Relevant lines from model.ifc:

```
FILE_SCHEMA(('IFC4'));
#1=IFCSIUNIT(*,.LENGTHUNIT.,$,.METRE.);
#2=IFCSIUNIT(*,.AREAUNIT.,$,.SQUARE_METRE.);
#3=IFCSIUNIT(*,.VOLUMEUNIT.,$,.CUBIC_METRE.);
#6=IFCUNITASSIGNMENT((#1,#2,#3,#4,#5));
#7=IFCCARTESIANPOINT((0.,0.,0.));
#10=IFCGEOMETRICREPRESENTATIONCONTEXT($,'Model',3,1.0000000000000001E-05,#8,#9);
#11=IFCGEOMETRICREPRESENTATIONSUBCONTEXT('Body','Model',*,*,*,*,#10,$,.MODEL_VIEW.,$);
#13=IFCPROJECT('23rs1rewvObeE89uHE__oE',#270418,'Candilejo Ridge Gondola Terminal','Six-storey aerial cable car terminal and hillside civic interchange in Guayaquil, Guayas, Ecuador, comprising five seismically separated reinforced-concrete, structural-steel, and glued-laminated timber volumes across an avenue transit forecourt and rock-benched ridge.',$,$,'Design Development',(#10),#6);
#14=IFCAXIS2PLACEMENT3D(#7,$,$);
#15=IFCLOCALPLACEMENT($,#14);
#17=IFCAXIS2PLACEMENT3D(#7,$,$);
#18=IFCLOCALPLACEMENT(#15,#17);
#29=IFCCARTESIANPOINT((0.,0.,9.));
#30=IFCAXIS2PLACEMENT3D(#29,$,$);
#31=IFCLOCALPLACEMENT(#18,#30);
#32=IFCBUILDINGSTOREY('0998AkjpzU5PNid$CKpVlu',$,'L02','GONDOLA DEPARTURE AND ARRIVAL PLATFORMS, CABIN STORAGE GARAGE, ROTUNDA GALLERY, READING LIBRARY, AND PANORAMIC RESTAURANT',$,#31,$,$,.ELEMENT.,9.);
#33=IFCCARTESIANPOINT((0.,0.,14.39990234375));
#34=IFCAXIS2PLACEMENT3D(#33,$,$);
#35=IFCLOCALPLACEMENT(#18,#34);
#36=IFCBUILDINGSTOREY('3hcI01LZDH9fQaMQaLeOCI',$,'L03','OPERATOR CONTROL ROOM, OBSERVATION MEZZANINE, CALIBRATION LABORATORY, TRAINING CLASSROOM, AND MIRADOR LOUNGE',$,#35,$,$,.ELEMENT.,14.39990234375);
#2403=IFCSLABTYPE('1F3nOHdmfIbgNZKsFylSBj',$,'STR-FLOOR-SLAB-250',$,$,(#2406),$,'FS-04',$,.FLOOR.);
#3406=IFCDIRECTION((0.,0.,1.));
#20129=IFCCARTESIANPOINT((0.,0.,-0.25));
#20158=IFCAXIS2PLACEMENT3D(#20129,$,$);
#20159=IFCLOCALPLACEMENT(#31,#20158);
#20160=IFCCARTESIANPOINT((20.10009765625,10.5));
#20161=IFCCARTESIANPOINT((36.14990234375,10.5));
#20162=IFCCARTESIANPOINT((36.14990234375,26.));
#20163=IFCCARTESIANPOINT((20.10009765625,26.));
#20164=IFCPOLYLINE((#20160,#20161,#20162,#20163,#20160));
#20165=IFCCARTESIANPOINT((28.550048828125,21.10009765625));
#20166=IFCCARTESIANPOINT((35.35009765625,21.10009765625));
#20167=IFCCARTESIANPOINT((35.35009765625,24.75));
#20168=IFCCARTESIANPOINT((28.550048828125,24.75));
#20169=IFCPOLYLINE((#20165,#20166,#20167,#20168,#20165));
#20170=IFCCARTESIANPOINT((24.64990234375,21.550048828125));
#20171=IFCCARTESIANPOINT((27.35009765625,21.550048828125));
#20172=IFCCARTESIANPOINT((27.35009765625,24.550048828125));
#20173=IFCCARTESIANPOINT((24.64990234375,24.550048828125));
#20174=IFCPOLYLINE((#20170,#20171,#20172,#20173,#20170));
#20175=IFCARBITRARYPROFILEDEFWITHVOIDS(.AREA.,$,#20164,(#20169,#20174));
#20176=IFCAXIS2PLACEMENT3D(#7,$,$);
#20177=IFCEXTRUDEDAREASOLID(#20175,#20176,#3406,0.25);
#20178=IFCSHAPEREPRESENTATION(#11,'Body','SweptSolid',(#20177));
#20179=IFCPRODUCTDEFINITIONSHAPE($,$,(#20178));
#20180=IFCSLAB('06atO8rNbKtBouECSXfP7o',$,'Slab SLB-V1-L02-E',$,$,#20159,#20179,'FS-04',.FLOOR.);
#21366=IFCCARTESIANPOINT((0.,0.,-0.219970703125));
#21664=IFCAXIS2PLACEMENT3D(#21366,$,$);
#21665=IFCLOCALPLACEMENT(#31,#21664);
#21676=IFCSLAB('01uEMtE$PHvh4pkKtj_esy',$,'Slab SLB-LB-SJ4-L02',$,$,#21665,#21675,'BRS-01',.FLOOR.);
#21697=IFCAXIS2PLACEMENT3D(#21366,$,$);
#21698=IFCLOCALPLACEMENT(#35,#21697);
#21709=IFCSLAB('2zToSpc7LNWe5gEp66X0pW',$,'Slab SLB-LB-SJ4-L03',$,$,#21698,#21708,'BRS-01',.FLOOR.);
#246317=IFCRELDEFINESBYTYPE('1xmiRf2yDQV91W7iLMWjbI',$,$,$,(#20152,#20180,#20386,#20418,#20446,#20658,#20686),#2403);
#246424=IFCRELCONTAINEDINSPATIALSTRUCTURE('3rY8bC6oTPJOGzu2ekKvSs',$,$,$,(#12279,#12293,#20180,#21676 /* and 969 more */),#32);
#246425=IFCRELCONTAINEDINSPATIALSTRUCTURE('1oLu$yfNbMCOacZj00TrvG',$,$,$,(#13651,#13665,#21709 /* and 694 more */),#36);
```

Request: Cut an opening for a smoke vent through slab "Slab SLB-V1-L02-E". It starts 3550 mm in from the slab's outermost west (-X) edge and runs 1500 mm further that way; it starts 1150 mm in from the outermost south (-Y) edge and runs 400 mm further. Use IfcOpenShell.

```python
import numpy as np
import ifcopenshell
import ifcopenshell.api.feature
import ifcopenshell.api.geometry
import ifcopenshell.api.root
import ifcopenshell.geom
import ifcopenshell.util.placement
import ifcopenshell.util.representation
import ifcopenshell.util.shape
import ifcopenshell.util.unit

model = ifcopenshell.open("model.ifc")
unit_scale = ifcopenshell.util.unit.calculate_unit_scale(model)
settings = ifcopenshell.geom.settings()


def volume(element):
    """Net volume in cubic metres, openings subtracted."""
    shape = ifcopenshell.geom.create_shape(settings, element)
    return ifcopenshell.util.shape.get_volume(shape.geometry)


slab = model.by_guid("06atO8rNbKtBouECSXfP7o")
before = volume(slab)

# Extent in the slab's own axes, in metres. The edges named are its -X and -Y sides.
slab_shape = ifcopenshell.geom.create_shape(settings, slab)
vertices = ifcopenshell.util.shape.get_vertices(slab_shape.geometry)
x_min, y_min, bottom = vertices.min(axis=0)
top = vertices[:, 2].max()

opening = ifcopenshell.api.root.create_entity(model, ifc_class="IfcOpeningElement", name="Smoke vent opening", predefined_type="OPENING")
context = ifcopenshell.util.representation.get_context(model, "Model", "Body", "MODEL_VIEW")
width, depth = 1.5, 0.4
outline = [(0.0, 0.0), (width, 0.0), (width, depth), (0.0, depth), (0.0, 0.0)]
# Overshoot both faces by 50 mm so the cut is clean.
shape = ifcopenshell.api.geometry.add_slab_representation(
    model, context=context, depth=top - bottom + 0.1, polyline=outline
)
ifcopenshell.api.geometry.assign_representation(model, product=opening, representation=shape)

matrix = ifcopenshell.util.placement.get_local_placement(slab.ObjectPlacement)
matrix[:, 3] = matrix @ np.append(np.array([x_min + 3.55, y_min + 1.15, bottom - 0.05]) / unit_scale, 1.0)
ifcopenshell.api.geometry.edit_object_placement(model, product=opening, matrix=matrix, is_si=False)
ifcopenshell.api.feature.add_feature(model, feature=opening, element=slab)

after = volume(slab)

print(f"slab volume {before:.3f} -> {after:.3f} m3")

model.write("model_rev.ifc")
```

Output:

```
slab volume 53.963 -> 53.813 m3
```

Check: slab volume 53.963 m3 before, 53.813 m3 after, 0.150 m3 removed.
